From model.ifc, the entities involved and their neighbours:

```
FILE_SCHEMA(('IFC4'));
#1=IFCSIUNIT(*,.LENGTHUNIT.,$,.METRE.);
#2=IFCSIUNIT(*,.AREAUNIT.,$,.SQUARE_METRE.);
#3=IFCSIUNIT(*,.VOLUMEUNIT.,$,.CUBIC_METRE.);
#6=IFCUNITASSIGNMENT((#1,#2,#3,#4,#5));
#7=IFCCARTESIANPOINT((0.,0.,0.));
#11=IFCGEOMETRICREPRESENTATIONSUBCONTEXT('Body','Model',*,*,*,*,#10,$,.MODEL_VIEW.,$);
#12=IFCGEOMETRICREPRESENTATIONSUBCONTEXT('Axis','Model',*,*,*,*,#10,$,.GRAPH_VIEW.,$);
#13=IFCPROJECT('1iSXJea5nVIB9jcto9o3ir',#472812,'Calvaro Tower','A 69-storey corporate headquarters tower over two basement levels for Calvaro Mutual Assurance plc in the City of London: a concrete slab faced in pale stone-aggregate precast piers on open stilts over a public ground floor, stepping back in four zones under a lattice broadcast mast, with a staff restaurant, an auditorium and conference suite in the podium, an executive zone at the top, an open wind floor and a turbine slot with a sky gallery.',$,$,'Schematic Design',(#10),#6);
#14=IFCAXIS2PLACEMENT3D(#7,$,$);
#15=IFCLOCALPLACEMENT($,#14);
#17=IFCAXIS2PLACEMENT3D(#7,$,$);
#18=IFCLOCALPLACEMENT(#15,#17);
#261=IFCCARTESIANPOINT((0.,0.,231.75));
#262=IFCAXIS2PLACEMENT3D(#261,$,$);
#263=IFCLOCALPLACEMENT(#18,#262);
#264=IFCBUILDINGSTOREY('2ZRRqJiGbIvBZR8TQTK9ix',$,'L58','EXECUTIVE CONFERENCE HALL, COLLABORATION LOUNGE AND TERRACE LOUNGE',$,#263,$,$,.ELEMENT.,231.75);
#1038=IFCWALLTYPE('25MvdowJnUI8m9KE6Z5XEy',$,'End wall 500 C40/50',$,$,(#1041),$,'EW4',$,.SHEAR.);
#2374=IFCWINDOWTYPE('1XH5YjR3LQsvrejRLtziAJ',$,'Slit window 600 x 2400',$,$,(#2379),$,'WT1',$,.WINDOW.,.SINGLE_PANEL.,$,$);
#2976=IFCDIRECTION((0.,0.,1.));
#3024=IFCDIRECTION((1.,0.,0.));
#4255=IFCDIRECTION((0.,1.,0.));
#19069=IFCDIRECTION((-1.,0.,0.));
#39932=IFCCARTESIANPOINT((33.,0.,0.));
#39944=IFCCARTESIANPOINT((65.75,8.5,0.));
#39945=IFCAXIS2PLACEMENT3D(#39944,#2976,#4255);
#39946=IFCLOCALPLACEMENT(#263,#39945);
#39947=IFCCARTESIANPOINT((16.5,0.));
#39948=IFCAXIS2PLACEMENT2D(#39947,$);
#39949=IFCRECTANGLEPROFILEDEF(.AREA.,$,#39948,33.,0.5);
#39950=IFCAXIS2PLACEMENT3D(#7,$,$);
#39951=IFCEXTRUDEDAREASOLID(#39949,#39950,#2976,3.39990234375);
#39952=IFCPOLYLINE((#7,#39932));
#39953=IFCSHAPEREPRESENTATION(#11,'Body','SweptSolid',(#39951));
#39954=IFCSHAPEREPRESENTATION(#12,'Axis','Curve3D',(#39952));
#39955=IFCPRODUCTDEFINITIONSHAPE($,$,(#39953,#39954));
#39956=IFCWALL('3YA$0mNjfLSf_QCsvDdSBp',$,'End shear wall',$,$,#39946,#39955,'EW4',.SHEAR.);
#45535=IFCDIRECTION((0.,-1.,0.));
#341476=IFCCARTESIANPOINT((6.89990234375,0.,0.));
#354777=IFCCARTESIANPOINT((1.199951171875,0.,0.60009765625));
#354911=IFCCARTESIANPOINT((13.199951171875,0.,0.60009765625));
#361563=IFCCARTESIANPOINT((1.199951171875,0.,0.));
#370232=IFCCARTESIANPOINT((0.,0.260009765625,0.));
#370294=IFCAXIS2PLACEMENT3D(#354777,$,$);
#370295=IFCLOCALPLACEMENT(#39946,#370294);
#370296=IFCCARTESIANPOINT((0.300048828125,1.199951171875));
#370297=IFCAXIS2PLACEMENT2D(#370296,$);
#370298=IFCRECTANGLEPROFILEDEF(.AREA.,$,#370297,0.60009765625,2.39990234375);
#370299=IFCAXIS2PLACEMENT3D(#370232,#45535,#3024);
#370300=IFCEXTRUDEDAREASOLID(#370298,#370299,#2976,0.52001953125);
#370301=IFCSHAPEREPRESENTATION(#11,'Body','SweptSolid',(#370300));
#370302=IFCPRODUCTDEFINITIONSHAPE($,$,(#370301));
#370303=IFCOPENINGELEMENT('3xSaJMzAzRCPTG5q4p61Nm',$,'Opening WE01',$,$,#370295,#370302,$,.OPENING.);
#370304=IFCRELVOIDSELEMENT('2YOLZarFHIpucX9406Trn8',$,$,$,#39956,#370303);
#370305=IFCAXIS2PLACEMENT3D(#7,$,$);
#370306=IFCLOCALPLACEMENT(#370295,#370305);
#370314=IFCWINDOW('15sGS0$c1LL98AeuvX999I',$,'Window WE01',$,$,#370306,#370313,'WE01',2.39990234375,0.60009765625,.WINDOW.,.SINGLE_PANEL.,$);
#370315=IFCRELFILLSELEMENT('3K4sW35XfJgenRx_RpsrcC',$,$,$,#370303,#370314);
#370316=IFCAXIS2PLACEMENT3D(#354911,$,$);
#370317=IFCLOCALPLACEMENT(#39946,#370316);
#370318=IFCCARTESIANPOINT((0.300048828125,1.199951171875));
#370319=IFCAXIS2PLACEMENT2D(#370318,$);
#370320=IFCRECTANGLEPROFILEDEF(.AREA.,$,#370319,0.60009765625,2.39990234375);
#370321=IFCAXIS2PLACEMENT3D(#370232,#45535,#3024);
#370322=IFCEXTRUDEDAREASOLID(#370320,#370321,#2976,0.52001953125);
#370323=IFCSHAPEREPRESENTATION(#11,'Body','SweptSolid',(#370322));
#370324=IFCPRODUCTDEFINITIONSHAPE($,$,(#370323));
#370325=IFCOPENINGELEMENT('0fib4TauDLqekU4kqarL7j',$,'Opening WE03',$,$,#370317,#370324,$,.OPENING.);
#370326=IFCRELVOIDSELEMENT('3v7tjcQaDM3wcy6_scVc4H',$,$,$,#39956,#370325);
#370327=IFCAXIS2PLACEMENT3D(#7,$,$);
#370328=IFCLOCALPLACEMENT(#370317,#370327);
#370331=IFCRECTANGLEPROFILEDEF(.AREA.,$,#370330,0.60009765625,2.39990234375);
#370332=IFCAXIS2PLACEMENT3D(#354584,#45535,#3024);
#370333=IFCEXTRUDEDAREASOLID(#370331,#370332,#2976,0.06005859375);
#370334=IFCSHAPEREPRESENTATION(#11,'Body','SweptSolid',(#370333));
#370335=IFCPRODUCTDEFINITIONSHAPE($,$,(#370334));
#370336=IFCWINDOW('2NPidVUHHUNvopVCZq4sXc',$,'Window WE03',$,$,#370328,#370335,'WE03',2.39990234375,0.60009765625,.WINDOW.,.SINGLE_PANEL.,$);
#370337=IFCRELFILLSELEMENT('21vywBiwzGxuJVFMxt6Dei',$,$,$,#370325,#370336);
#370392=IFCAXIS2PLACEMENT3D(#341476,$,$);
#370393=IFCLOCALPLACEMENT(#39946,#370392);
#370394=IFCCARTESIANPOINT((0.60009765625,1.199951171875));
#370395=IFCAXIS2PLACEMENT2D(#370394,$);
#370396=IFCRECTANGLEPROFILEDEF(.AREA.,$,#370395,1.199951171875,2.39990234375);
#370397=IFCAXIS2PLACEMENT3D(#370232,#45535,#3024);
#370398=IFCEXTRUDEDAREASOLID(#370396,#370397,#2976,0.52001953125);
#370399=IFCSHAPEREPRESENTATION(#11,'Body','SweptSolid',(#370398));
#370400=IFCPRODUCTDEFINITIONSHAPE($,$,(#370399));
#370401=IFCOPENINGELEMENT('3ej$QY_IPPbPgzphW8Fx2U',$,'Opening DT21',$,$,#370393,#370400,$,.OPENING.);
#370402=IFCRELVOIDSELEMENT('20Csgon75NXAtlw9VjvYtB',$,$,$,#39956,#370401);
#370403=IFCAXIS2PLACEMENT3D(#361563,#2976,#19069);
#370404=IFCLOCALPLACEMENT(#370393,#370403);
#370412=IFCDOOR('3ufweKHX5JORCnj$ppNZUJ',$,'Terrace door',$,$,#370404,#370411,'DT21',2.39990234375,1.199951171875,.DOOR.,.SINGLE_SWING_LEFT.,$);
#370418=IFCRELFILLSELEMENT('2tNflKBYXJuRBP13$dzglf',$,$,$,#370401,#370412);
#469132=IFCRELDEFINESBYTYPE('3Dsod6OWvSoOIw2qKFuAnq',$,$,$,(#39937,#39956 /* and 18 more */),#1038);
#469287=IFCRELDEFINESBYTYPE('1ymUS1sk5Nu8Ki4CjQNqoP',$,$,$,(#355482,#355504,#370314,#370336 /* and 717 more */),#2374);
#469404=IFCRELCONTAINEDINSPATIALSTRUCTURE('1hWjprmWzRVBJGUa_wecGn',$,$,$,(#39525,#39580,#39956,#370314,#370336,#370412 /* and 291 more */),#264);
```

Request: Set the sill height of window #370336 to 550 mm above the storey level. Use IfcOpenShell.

```python
import numpy as np
import ifcopenshell
import ifcopenshell.api.geometry
import ifcopenshell.geom
import ifcopenshell.util.element
import ifcopenshell.util.placement
import ifcopenshell.util.shape
import ifcopenshell.util.unit

model = ifcopenshell.open("model.ifc")
unit_scale = ifcopenshell.util.unit.calculate_unit_scale(model)

window = model.by_guid("2NPidVUHHUNvopVCZq4sXc")
opening = window.FillsVoids[0].RelatingOpeningElement
storey = ifcopenshell.util.element.get_container(window, ifc_class="IfcBuildingStorey")
level = ifcopenshell.util.placement.get_local_placement(storey.ObjectPlacement)[2, 3]

# The opening's origin need not be at the sill, so measure its lowest point.
shape = ifcopenshell.geom.create_shape(ifcopenshell.geom.settings(), opening)
bottom = ifcopenshell.util.shape.get_shape_bottom_elevation(shape, shape.geometry) / unit_scale
dz = level + 0.55 - bottom

shift = np.array([0.0, 0.0, dz])
# The window is placed relative to its opening, so it follows when the opening moves.
matrix = ifcopenshell.util.placement.get_local_placement(opening.ObjectPlacement)
matrix[:3, 3] += shift
ifcopenshell.api.geometry.edit_object_placement(
    model, product=opening, matrix=matrix, is_si=False, should_transform_children=True
)

print(f"moved by {dz * unit_scale:+.3f} m")

model.write("model_rev.ifc")
```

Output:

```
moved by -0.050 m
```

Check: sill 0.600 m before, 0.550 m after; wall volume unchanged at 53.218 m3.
